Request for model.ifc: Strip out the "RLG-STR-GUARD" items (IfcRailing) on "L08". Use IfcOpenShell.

First a look at what the model holds.

```python
import ifcopenshell
import ifcopenshell.util.element

model = ifcopenshell.open("model.ifc")
print(model.schema)
storey = next(s for s in model.by_type("IfcBuildingStorey") if s.Name == "L08")
railings = [e for e in ifcopenshell.util.element.get_decomposition(storey) if e.is_a("IfcRailing")]
seen = {}
for e in railings:
    element_type = ifcopenshell.util.element.get_type(e)
    name = element_type.Name if element_type not in (None, e) else None
    seen[name] = seen.get(name, 0) + 1
for name, count in sorted(seen.items(), key=str):
    print(count, "x", name)
```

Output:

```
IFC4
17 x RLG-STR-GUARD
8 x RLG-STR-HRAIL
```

```python
import ifcopenshell
import ifcopenshell.api.root
import ifcopenshell.util.element

model = ifcopenshell.open("model.ifc")

storey = next(s for s in model.by_type("IfcBuildingStorey") if s.Name == "L08")
railings = [e for e in ifcopenshell.util.element.get_decomposition(storey) if e.is_a("IfcRailing")]
targets = [e for e in railings if (t := ifcopenshell.util.element.get_type(e)) not in (None, e) and t.Name == "RLG-STR-GUARD"]

for e in targets:
    ifcopenshell.api.root.remove_product(model, product=e)
print(len(targets), "removed")

model.write("model_edited.ifc")
```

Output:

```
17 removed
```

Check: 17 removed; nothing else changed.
